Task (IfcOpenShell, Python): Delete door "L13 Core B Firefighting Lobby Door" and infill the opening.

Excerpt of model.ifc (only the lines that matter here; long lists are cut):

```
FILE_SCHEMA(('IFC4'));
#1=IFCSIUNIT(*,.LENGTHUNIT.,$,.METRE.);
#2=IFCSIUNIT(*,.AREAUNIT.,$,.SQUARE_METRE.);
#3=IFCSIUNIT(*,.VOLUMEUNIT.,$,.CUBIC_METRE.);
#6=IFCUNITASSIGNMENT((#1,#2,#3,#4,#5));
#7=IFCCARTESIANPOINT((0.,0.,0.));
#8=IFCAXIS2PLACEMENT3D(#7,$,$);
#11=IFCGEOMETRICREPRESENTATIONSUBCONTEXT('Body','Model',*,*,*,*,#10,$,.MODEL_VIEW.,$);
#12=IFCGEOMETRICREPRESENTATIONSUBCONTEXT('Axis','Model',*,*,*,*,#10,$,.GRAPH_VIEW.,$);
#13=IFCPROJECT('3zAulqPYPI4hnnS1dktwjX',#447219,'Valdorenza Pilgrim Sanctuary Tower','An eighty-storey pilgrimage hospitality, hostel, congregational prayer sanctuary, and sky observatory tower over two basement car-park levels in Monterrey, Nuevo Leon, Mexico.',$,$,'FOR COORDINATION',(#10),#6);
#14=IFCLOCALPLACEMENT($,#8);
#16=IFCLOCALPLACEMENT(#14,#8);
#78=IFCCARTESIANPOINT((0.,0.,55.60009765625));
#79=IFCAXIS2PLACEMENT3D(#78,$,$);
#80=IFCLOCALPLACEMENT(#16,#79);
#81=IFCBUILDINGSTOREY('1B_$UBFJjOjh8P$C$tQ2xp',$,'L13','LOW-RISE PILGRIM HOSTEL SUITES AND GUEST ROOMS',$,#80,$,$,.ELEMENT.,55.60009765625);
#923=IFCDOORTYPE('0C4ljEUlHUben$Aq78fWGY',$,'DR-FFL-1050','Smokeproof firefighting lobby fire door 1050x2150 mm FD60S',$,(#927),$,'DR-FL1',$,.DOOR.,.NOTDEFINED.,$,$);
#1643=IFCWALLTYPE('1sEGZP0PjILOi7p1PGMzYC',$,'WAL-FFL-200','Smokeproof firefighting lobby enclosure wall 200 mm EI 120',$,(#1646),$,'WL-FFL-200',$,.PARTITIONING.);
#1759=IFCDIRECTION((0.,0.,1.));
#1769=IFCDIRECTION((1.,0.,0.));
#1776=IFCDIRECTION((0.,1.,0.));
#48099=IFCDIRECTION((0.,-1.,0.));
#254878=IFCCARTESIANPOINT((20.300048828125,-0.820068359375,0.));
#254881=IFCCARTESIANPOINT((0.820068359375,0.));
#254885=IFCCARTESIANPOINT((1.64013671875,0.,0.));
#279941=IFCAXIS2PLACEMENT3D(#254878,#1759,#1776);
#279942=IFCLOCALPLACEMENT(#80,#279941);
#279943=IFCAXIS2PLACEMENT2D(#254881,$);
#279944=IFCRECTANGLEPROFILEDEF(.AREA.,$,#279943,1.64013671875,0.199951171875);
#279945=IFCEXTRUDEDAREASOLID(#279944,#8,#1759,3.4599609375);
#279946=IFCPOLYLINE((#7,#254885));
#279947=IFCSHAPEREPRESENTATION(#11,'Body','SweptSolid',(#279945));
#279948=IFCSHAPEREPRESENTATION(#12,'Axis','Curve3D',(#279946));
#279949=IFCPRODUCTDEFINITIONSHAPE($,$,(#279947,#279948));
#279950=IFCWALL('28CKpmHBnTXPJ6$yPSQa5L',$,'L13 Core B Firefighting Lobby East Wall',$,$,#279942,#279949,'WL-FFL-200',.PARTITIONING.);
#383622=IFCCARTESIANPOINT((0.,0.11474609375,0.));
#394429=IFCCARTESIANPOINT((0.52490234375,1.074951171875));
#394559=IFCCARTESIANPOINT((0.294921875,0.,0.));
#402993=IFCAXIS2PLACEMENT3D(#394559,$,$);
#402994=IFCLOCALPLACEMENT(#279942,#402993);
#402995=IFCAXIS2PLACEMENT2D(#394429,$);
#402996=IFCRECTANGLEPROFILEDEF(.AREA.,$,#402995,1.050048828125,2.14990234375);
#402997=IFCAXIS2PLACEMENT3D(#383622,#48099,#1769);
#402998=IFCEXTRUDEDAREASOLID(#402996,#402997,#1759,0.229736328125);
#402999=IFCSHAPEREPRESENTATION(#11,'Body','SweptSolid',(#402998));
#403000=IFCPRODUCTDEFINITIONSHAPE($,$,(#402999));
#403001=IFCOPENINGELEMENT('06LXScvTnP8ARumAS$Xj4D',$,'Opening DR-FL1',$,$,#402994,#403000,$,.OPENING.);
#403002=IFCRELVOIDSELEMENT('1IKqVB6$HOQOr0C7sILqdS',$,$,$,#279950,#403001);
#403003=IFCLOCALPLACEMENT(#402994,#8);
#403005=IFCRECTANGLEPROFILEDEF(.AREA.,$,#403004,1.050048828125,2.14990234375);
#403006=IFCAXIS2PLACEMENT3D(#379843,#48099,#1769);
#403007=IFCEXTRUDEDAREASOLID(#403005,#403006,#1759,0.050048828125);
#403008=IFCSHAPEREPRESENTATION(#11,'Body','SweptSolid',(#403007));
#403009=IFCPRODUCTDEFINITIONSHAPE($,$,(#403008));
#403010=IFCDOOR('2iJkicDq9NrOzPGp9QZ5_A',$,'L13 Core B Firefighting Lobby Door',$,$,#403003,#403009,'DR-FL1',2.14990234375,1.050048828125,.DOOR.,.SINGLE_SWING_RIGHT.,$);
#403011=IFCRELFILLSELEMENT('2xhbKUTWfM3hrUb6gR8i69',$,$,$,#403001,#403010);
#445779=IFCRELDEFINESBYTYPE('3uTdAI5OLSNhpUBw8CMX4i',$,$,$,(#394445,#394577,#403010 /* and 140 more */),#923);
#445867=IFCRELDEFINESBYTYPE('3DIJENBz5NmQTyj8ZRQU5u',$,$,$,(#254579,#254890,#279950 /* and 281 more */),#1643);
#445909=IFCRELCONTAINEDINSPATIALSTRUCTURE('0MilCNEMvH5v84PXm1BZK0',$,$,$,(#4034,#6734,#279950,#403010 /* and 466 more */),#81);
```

```python
import ifcopenshell
import ifcopenshell.api.feature
import ifcopenshell.api.root
import ifcopenshell.geom
import ifcopenshell.util.shape

model = ifcopenshell.open("model.ifc")
settings = ifcopenshell.geom.settings()


def volume(element):
    """Net volume in cubic metres, openings subtracted."""
    shape = ifcopenshell.geom.create_shape(settings, element)
    return ifcopenshell.util.shape.get_volume(shape.geometry)


door = model.by_guid("2iJkicDq9NrOzPGp9QZ5_A")
opening = door.FillsVoids[0].RelatingOpeningElement
wall = opening.VoidsElements[0].RelatingBuildingElement
before = volume(wall)

ifcopenshell.api.root.remove_product(model, product=door)
ifcopenshell.api.feature.remove_feature(model, feature=opening)

after = volume(wall)

print(f"wall volume {before:.3f} -> {after:.3f} m3")

model.write("model_edited.ifc")
```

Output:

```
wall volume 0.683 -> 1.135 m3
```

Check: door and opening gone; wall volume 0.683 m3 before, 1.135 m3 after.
